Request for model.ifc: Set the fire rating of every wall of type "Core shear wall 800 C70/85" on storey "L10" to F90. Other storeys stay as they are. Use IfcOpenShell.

First a look at what the model holds.

```python
import ifcopenshell
import ifcopenshell.util.element

model = ifcopenshell.open("model.ifc")
print(model.schema)
storey = next(s for s in model.by_type("IfcBuildingStorey") if s.Name == "L10")
walls = [e for e in ifcopenshell.util.element.get_decomposition(storey) if e.is_a("IfcWall")]
seen = {}
for e in walls:
    element_type = ifcopenshell.util.element.get_type(e)
    key = (element_type.Name if element_type != e and element_type else None, ifcopenshell.util.element.get_pset(e, "Pset_WallCommon", "FireRating"))
    seen[key] = seen.get(key, 0) + 1
for (name, value), count in sorted(seen.items(), key=str):
    print(count, "x", name, "|", value)
```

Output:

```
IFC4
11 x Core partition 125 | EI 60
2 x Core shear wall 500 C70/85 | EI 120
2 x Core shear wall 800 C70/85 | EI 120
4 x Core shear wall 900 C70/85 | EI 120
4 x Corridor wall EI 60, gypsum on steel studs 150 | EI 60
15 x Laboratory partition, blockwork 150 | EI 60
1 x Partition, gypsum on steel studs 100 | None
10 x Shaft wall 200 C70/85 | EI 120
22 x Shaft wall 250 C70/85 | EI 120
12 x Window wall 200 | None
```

```python
import ifcopenshell
import ifcopenshell.api.pset
import ifcopenshell.util.element

model = ifcopenshell.open("model.ifc")

storey = next(s for s in model.by_type("IfcBuildingStorey") if s.Name == "L10")
walls = [e for e in ifcopenshell.util.element.get_decomposition(storey) if e.is_a("IfcWall")]

count = 0
for e in walls:
    element_type = ifcopenshell.util.element.get_type(e)
    if element_type in (None, e) or element_type.Name != "Core shear wall 800 C70/85":
        continue
    found = ifcopenshell.util.element.get_pset(e, "Pset_WallCommon", should_inherit=False)
    if found:
        pset = model.by_id(found["id"])
        if len(ifcopenshell.util.element.get_elements_by_pset(pset)) > 1:
            pset = ifcopenshell.api.pset.unshare_pset(model, products=[e], pset=pset)[0]
    else:
        pset = ifcopenshell.api.pset.add_pset(model, product=e, name="Pset_WallCommon")
    ifcopenshell.api.pset.edit_pset(model, pset=pset, properties={"FireRating": "F90"})
    count += 1

print(count, "walls updated")

model.write("model_rev.ifc")
```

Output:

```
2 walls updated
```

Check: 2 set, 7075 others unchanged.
